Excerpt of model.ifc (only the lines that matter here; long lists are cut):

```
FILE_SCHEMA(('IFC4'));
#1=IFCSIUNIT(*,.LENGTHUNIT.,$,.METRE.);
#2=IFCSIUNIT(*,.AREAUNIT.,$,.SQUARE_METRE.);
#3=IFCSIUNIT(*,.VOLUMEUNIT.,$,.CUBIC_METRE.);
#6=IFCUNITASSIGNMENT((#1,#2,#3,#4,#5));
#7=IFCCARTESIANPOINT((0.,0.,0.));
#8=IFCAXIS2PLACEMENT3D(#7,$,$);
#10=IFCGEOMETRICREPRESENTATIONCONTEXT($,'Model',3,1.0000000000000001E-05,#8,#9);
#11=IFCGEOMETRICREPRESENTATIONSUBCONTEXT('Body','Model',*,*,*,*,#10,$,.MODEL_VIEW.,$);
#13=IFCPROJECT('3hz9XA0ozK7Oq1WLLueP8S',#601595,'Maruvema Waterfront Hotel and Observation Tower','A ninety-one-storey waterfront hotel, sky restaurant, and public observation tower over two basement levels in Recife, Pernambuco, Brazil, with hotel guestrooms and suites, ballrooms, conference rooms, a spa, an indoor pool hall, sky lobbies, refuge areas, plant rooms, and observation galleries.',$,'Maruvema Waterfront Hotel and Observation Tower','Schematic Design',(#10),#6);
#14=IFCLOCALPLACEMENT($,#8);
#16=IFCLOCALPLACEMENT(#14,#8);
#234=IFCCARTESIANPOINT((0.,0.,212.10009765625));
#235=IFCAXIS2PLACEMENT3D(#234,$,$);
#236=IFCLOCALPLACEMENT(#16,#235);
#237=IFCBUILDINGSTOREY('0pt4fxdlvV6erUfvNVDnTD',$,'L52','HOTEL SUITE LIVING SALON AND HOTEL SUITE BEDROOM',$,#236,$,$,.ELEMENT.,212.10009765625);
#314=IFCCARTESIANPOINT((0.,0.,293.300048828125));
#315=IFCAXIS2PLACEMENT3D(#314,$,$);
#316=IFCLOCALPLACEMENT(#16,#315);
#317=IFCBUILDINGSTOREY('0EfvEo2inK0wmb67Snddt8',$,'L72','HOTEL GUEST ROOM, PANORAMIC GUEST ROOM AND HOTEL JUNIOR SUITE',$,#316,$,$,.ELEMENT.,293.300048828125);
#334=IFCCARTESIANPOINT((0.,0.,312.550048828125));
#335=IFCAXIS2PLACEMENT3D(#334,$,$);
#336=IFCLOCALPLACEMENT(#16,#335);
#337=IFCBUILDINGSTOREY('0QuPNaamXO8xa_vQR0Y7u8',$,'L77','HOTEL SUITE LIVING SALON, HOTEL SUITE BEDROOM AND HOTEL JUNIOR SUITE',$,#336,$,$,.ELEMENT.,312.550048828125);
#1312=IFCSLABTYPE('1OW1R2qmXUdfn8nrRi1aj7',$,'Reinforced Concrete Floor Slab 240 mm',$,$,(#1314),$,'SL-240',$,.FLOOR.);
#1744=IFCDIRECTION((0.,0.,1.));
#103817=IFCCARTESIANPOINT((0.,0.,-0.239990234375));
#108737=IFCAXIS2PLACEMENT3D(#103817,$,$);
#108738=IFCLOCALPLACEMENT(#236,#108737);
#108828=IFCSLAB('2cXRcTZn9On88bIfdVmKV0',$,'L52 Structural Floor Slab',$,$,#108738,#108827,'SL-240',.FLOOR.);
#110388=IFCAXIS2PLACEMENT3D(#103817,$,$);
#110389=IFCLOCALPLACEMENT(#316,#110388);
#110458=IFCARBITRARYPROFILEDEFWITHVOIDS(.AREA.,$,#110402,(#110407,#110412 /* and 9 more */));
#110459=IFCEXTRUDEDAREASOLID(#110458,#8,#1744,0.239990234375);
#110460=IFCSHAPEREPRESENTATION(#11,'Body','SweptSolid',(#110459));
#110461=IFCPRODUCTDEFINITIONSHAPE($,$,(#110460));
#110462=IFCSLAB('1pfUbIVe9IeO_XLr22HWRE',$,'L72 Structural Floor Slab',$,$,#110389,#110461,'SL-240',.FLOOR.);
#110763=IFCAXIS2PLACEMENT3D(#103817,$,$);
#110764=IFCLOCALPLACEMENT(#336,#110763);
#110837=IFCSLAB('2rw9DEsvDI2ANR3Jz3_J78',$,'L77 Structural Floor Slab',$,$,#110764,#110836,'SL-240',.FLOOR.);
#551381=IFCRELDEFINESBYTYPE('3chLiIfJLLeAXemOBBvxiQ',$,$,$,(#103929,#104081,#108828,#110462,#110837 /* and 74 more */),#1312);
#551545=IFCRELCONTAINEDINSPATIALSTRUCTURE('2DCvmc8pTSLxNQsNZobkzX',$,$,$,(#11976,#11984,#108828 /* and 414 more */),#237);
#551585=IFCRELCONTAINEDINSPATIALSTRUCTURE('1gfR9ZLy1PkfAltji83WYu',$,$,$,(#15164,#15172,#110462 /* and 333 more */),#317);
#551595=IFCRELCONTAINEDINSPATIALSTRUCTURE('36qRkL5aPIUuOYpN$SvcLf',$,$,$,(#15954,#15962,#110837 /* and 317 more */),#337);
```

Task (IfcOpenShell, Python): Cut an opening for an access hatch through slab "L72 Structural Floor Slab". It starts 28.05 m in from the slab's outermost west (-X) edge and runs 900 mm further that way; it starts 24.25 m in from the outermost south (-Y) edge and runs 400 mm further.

```python
import numpy as np
import ifcopenshell
import ifcopenshell.api.feature
import ifcopenshell.api.geometry
import ifcopenshell.api.root
import ifcopenshell.geom
import ifcopenshell.util.placement
import ifcopenshell.util.representation
import ifcopenshell.util.shape
import ifcopenshell.util.unit

model = ifcopenshell.open("model.ifc")
unit_scale = ifcopenshell.util.unit.calculate_unit_scale(model)
settings = ifcopenshell.geom.settings()


def volume(element):
    """Net volume in cubic metres, openings subtracted."""
    shape = ifcopenshell.geom.create_shape(settings, element)
    return ifcopenshell.util.shape.get_volume(shape.geometry)


slab = model.by_guid("1pfUbIVe9IeO_XLr22HWRE")
before = volume(slab)

# Extent in the slab's own axes, in metres. The edges named are its -X and -Y sides.
slab_shape = ifcopenshell.geom.create_shape(settings, slab)
vertices = ifcopenshell.util.shape.get_vertices(slab_shape.geometry)
x_min, y_min, bottom = vertices.min(axis=0)
top = vertices[:, 2].max()

opening = ifcopenshell.api.root.create_entity(model, ifc_class="IfcOpeningElement", name="Access hatch opening", predefined_type="OPENING")
context = ifcopenshell.util.representation.get_context(model, "Model", "Body", "MODEL_VIEW")
width, depth = 0.9, 0.4
outline = [(0.0, 0.0), (width, 0.0), (width, depth), (0.0, depth), (0.0, 0.0)]
# Overshoot both faces by 50 mm so the cut is clean.
shape = ifcopenshell.api.geometry.add_slab_representation(
    model, context=context, depth=top - bottom + 0.1, polyline=outline
)
ifcopenshell.api.geometry.assign_representation(model, product=opening, representation=shape)

matrix = ifcopenshell.util.placement.get_local_placement(slab.ObjectPlacement)
matrix[:, 3] = matrix @ np.append(np.array([x_min + 28.05, y_min + 24.25, bottom - 0.05]) / unit_scale, 1.0)
ifcopenshell.api.geometry.edit_object_placement(model, product=opening, matrix=matrix, is_si=False)
ifcopenshell.api.feature.add_feature(model, feature=opening, element=slab)

after = volume(slab)

print(f"slab volume {before:.3f} -> {after:.3f} m3")

model.write("model_rev.ifc")
```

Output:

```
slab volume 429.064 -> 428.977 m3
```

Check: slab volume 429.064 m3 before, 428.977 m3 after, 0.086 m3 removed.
